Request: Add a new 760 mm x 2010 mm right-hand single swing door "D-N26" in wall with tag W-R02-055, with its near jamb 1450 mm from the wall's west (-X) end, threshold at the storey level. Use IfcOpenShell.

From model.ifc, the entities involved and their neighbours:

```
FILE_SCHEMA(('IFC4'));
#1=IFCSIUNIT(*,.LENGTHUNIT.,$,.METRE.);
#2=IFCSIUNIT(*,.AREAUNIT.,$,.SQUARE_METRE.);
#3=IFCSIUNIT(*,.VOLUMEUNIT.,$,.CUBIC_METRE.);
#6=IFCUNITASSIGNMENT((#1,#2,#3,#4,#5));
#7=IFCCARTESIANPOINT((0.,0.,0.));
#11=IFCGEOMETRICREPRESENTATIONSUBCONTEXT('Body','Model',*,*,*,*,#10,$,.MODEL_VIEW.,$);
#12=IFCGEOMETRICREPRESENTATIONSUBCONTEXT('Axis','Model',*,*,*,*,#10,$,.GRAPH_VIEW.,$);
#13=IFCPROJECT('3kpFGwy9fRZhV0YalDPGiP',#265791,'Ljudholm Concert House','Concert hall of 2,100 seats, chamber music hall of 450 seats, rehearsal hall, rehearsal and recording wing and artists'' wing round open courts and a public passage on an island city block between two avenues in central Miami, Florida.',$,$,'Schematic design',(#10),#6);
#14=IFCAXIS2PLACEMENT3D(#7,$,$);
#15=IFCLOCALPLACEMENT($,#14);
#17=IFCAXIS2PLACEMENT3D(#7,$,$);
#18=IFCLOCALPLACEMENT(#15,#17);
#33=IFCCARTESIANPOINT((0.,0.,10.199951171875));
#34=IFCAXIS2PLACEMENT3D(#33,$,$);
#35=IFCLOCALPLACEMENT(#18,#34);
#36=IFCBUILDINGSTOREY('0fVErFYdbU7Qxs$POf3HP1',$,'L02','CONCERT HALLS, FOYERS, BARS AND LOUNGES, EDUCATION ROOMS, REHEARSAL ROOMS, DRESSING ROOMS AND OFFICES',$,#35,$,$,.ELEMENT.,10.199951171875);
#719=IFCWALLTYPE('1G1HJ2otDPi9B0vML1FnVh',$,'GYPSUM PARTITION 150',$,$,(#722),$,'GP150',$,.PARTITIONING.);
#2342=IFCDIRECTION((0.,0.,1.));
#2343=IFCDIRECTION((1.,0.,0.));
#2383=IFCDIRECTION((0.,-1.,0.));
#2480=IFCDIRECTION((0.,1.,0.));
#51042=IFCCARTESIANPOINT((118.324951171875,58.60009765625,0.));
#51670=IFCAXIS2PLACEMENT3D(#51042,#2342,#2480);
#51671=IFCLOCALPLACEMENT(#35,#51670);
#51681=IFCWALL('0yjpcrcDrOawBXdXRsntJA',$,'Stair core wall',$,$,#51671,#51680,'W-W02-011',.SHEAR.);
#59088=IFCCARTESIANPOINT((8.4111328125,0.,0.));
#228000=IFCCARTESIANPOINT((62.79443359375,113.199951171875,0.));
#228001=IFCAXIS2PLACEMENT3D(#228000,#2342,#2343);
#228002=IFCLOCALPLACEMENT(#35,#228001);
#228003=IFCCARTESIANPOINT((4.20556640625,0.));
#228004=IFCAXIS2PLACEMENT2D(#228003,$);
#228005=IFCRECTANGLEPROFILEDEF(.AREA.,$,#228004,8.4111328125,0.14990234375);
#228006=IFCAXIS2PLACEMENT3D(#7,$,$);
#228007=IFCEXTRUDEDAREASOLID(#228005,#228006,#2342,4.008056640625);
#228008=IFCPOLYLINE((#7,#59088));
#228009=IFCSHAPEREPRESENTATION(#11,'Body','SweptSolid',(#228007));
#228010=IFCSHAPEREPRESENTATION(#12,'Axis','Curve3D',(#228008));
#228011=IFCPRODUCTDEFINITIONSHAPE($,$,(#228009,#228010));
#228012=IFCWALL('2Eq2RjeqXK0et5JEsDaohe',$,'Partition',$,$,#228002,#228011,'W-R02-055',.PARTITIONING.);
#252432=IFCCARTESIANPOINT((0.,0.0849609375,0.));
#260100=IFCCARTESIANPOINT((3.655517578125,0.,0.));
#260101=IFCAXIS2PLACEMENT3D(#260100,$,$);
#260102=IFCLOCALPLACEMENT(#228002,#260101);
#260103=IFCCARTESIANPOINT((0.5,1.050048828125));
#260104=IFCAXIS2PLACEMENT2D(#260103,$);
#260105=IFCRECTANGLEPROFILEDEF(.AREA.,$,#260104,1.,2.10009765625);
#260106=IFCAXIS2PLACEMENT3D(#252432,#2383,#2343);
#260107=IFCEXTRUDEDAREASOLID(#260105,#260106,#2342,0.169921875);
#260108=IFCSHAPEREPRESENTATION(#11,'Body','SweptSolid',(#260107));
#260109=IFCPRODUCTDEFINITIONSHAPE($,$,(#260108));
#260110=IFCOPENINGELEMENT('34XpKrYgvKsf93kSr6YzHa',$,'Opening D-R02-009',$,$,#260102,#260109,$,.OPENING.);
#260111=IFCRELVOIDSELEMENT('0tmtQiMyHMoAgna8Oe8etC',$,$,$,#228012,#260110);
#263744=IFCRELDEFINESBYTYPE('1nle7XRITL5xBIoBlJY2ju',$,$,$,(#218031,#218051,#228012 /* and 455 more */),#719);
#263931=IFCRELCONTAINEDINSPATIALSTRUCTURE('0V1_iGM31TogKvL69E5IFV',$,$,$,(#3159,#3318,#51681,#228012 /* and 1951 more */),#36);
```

```python
import numpy as np
import ifcopenshell
import ifcopenshell.api.feature
import ifcopenshell.api.geometry
import ifcopenshell.api.root
import ifcopenshell.api.spatial
import ifcopenshell.geom
import ifcopenshell.util.element
import ifcopenshell.util.placement
import ifcopenshell.util.representation
import ifcopenshell.util.shape
import ifcopenshell.util.unit

model = ifcopenshell.open("model.ifc")
unit_scale = ifcopenshell.util.unit.calculate_unit_scale(model)
settings = ifcopenshell.geom.settings()


def volume(element):
    """Net volume in cubic metres, openings subtracted."""
    shape = ifcopenshell.geom.create_shape(settings, element)
    return ifcopenshell.util.shape.get_volume(shape.geometry)


wall = model.by_guid("2Eq2RjeqXK0et5JEsDaohe")
storey = ifcopenshell.util.element.get_container(wall, ifc_class="IfcBuildingStorey")
context = ifcopenshell.util.representation.get_context(model, "Model", "Body", "MODEL_VIEW")
before = volume(wall)

width, height, from_end, sill = 0.76, 2.01, 1.45, 0.0  # metres

# The wall runs along its own X axis, and the end named is its -X end.
wall_shape = ifcopenshell.geom.create_shape(settings, wall)
x, y, z = ifcopenshell.util.shape.get_vertices(wall_shape.geometry).T
start = x.min() + from_end
face, thickness = float(y.min()), float(y.max() - y.min())
wall_matrix = ifcopenshell.util.placement.get_local_placement(wall.ObjectPlacement)
level = ifcopenshell.util.placement.get_local_placement(storey.ObjectPlacement)[2, 3]


def in_wall(x, y):
    """Placement at x, y metres in the wall's axes, at sill height."""
    matrix = wall_matrix.copy()
    matrix[:, 3] = wall_matrix @ np.array([x / unit_scale, y / unit_scale, 0.0, 1.0])
    matrix[2, 3] = level + sill / unit_scale
    return matrix


# Opening: a box that overshoots both wall faces by 50 mm.
opening = ifcopenshell.api.root.create_entity(model, ifc_class="IfcOpeningElement", predefined_type="OPENING")
box = ifcopenshell.api.geometry.add_wall_representation(
    model, context=context, length=width, height=height, thickness=thickness + 0.1
)
ifcopenshell.api.geometry.assign_representation(model, product=opening, representation=box)
ifcopenshell.api.geometry.edit_object_placement(model, product=opening, matrix=in_wall(start, face - 0.05), is_si=False)
ifcopenshell.api.feature.add_feature(model, feature=opening, element=wall)

door = ifcopenshell.api.root.create_entity(model, ifc_class="IfcDoor", name="D-N26", predefined_type="DOOR")
door.OverallWidth, door.OverallHeight = width / unit_scale, height / unit_scale
door.OperationType = "SINGLE_SWING_RIGHT"
body = ifcopenshell.api.geometry.add_door_representation(
    model,
    context=context,
    overall_width=door.OverallWidth,
    overall_height=door.OverallHeight,
    operation_type="SINGLE_SWING_RIGHT",
    lining_properties={"LiningDepth": thickness / unit_scale, "ThresholdDepth": thickness / unit_scale},
)
ifcopenshell.api.geometry.assign_representation(model, product=door, representation=body)
ifcopenshell.api.spatial.assign_container(model, products=[door], relating_structure=storey)
ifcopenshell.api.feature.add_filling(model, opening=opening, element=door)

# The lining spans the wall, so the door starts at the wall face.
ifcopenshell.api.geometry.edit_object_placement(model, product=door, matrix=in_wall(start, face), is_si=False)

after = volume(wall)

print(f"wall volume {before:.3f} -> {after:.3f} m3")

model.write("model_v2.ifc")
```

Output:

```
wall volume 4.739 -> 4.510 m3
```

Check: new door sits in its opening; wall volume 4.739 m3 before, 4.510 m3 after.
